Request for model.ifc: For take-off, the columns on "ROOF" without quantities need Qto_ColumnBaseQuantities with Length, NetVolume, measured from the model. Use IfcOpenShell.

First a look at what the model holds.

```python
import ifcopenshell
import ifcopenshell.util.element
import ifcopenshell.util.unit

model = ifcopenshell.open("model.ifc")
print(model.schema)
for unit_type in ("LENGTHUNIT", "AREAUNIT", "VOLUMEUNIT"):
    print(unit_type, ifcopenshell.util.unit.calculate_unit_scale(model, unit_type))
storey = next(s for s in model.by_type("IfcBuildingStorey") if s.Name == "ROOF")
columns = [e for e in ifcopenshell.util.element.get_decomposition(storey) if e.is_a("IfcColumn")]
for e in sorted(columns, key=lambda e: e.id()):
    print(e.id(), e.is_a(), e.Name, list(ifcopenshell.util.element.get_psets(e, qtos_only=True)), sep=" | ")
```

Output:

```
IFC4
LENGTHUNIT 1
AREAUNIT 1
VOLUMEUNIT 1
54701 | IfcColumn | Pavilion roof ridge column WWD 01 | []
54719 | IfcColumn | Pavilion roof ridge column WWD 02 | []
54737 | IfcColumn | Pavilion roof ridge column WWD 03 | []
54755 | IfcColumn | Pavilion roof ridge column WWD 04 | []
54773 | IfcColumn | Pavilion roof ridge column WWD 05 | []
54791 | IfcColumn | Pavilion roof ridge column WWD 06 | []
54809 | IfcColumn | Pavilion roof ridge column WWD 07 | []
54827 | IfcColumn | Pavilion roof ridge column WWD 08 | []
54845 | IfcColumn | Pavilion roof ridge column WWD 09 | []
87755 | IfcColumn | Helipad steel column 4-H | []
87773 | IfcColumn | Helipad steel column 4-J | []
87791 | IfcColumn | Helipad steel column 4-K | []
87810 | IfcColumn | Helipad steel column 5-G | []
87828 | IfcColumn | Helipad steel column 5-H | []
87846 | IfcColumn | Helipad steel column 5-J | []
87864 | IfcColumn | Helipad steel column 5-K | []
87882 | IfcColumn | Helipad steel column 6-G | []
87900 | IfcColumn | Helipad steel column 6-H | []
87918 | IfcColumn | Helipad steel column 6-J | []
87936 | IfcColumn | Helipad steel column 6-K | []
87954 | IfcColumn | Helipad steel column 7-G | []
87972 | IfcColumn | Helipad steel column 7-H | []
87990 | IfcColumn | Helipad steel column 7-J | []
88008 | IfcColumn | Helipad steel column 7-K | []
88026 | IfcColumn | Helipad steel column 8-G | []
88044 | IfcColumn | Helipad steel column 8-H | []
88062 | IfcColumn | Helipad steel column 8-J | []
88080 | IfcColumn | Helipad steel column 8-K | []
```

```python
import ifcopenshell
import ifcopenshell.api.pset
import ifcopenshell.geom
import ifcopenshell.util.element
import ifcopenshell.util.shape
import ifcopenshell.util.unit

model = ifcopenshell.open("model.ifc")
unit_scale = ifcopenshell.util.unit.calculate_unit_scale(model)
volume_scale = ifcopenshell.util.unit.calculate_unit_scale(model, "VOLUMEUNIT")
settings = ifcopenshell.geom.settings()

storey = next(s for s in model.by_type("IfcBuildingStorey") if s.Name == "ROOF")
columns = [e for e in ifcopenshell.util.element.get_decomposition(storey) if e.is_a("IfcColumn")]

for e in sorted(columns, key=lambda e: e.id()):
    if ifcopenshell.util.element.get_psets(e, qtos_only=True, should_inherit=False):
        continue
    # Geometry comes back in metres, in the element's own axes.
    shape = ifcopenshell.geom.create_shape(settings, e)
    values = {
        "Length": ifcopenshell.util.shape.get_z(shape.geometry) / unit_scale,
        "NetVolume": ifcopenshell.util.shape.get_volume(shape.geometry) / volume_scale,
    }
    qto = ifcopenshell.api.pset.add_qto(model, product=e, name="Qto_ColumnBaseQuantities")
    ifcopenshell.api.pset.edit_qto(model, qto=qto, properties=values)
    print(e.id(), {k: round(v, 3) for k, v in values.items()})

model.write("model_updated.ifc")
```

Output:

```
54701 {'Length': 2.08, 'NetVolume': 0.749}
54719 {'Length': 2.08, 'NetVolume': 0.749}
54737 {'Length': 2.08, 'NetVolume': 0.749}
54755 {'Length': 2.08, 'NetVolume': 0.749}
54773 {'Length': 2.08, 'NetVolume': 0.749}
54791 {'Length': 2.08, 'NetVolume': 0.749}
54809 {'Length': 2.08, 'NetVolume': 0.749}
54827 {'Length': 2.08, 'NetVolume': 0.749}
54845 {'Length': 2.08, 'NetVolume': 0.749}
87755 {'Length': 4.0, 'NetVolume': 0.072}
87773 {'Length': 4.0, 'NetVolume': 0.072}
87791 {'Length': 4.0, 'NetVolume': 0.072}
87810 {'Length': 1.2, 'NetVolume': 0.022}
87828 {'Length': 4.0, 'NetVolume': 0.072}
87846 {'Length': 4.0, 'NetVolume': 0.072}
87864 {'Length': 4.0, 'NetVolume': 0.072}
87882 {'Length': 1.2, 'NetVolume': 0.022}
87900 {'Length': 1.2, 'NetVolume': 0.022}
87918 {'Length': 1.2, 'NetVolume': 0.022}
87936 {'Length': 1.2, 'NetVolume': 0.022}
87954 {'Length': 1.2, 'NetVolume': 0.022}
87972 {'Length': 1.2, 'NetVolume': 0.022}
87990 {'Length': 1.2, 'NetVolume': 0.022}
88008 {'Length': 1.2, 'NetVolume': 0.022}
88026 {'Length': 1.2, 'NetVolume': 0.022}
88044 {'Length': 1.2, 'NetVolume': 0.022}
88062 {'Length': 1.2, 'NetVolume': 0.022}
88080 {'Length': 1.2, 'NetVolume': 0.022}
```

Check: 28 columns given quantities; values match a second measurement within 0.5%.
